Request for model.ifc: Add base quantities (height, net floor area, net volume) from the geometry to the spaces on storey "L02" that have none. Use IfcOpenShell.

First a look at what the model holds.

```python
import ifcopenshell
import ifcopenshell.util.element
import ifcopenshell.util.unit

model = ifcopenshell.open("model.ifc")
print(model.schema)
for unit_type in ("LENGTHUNIT", "AREAUNIT", "VOLUMEUNIT"):
    print(unit_type, ifcopenshell.util.unit.calculate_unit_scale(model, unit_type))
storey = next(s for s in model.by_type("IfcBuildingStorey") if s.Name == "L02")
spaces = [e for e in ifcopenshell.util.element.get_decomposition(storey) if e.is_a("IfcSpace")]
for e in sorted(spaces, key=lambda e: e.id()):
    print(e.id(), e.is_a(), e.Name, list(ifcopenshell.util.element.get_psets(e, qtos_only=True)), sep=" | ")
```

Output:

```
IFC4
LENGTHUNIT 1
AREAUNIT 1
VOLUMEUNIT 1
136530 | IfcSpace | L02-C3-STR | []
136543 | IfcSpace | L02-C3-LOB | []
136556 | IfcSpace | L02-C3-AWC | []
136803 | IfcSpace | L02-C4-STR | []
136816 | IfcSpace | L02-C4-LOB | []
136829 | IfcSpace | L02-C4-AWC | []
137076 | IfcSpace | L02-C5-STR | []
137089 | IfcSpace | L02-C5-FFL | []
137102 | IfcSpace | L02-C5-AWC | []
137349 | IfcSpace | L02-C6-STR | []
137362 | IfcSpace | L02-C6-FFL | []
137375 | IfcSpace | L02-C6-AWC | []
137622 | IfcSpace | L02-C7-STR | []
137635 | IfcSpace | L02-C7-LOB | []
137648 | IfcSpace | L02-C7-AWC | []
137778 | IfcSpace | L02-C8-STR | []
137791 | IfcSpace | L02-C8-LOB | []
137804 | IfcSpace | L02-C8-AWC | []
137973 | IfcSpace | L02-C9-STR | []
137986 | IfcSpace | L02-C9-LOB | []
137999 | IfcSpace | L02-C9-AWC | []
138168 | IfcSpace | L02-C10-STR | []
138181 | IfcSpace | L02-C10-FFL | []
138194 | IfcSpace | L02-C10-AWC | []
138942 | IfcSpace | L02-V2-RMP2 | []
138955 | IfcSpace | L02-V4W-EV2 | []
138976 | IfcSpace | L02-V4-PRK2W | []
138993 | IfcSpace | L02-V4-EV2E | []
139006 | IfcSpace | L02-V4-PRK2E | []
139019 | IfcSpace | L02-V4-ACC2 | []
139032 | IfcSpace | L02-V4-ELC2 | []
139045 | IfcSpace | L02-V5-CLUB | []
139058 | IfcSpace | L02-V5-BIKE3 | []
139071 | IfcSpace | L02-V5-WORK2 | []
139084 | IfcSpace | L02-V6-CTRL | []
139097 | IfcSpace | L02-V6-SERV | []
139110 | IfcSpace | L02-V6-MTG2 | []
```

```python
import ifcopenshell
import ifcopenshell.api.pset
import ifcopenshell.geom
import ifcopenshell.util.element
import ifcopenshell.util.shape
import ifcopenshell.util.unit

model = ifcopenshell.open("model.ifc")
unit_scale = ifcopenshell.util.unit.calculate_unit_scale(model)
area_scale = ifcopenshell.util.unit.calculate_unit_scale(model, "AREAUNIT")
volume_scale = ifcopenshell.util.unit.calculate_unit_scale(model, "VOLUMEUNIT")
settings = ifcopenshell.geom.settings()

storey = next(s for s in model.by_type("IfcBuildingStorey") if s.Name == "L02")
spaces = [e for e in ifcopenshell.util.element.get_decomposition(storey) if e.is_a("IfcSpace")]

for e in sorted(spaces, key=lambda e: e.id()):
    if ifcopenshell.util.element.get_psets(e, qtos_only=True, should_inherit=False):
        continue
    # Geometry comes back in metres, in the element's own axes.
    shape = ifcopenshell.geom.create_shape(settings, e)
    values = {
        "Height": ifcopenshell.util.shape.get_z(shape.geometry) / unit_scale,
        "NetFloorArea": ifcopenshell.util.shape.get_footprint_area(shape.geometry) / area_scale,
        "NetVolume": ifcopenshell.util.shape.get_volume(shape.geometry) / volume_scale,
    }
    qto = ifcopenshell.api.pset.add_qto(model, product=e, name="Qto_SpaceBaseQuantities")
    ifcopenshell.api.pset.edit_qto(model, qto=qto, properties=values)
    print(e.id(), {k: round(v, 3) for k, v in values.items()})

model.write("model_rev.ifc")
```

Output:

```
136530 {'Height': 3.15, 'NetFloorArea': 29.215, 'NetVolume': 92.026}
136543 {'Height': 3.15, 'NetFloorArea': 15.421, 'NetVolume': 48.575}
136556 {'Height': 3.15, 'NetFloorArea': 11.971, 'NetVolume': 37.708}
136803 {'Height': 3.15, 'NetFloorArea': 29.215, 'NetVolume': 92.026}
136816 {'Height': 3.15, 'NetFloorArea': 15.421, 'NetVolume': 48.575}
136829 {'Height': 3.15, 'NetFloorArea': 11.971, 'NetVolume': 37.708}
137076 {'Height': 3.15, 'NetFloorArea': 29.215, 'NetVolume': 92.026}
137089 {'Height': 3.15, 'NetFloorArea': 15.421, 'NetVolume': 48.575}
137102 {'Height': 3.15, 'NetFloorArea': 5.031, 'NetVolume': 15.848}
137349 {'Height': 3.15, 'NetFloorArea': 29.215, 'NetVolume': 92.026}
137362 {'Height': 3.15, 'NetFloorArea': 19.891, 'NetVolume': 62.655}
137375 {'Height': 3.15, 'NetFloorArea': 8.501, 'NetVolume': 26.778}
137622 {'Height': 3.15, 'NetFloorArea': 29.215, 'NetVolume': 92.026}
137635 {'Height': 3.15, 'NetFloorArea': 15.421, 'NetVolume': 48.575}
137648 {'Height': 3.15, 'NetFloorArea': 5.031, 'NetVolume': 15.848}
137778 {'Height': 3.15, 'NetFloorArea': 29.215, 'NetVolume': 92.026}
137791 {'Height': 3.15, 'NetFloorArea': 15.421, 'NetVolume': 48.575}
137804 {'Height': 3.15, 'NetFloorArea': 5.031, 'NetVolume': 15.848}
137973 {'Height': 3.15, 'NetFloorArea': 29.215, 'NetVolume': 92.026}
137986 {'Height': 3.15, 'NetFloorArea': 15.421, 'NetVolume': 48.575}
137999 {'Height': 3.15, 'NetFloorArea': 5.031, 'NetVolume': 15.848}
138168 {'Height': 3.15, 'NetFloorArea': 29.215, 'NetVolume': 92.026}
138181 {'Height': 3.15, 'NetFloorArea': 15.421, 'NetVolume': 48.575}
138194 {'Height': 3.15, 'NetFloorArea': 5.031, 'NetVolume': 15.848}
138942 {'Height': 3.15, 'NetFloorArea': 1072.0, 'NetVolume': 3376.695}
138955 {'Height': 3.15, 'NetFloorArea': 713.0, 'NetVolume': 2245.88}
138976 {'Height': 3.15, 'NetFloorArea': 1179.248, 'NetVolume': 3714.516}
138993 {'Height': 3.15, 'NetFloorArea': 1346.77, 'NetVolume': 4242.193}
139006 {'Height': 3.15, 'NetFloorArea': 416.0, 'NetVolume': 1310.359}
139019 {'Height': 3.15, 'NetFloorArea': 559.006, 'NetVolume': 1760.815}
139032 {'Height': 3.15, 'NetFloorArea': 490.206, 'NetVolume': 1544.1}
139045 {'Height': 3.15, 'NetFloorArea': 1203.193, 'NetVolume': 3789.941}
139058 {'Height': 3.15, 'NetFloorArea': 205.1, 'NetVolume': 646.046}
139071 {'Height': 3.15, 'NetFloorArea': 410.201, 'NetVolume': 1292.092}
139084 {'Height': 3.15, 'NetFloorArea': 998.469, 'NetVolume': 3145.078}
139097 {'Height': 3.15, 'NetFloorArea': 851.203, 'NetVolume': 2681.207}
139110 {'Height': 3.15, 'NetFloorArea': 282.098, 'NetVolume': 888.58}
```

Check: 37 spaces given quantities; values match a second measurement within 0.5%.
